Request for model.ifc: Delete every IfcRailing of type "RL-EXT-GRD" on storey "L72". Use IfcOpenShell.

First a look at what the model holds.

```python
import ifcopenshell
import ifcopenshell.util.element

model = ifcopenshell.open("model.ifc")
print(model.schema)
storey = next(s for s in model.by_type("IfcBuildingStorey") if s.Name == "L72")
railings = [e for e in ifcopenshell.util.element.get_decomposition(storey) if e.is_a("IfcRailing")]
seen = {}
for e in railings:
    element_type = ifcopenshell.util.element.get_type(e)
    name = element_type.Name if element_type not in (None, e) else None
    seen[name] = seen.get(name, 0) + 1
for name, count in sorted(seen.items(), key=str):
    print(count, "x", name)
```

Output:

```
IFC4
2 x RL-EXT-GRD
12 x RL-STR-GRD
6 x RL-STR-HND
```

```python
import ifcopenshell
import ifcopenshell.api.root
import ifcopenshell.util.element

model = ifcopenshell.open("model.ifc")

storey = next(s for s in model.by_type("IfcBuildingStorey") if s.Name == "L72")
railings = [e for e in ifcopenshell.util.element.get_decomposition(storey) if e.is_a("IfcRailing")]
targets = [e for e in railings if (t := ifcopenshell.util.element.get_type(e)) not in (None, e) and t.Name == "RL-EXT-GRD"]

for e in targets:
    ifcopenshell.api.root.remove_product(model, product=e)
print(len(targets), "removed")

model.write("model_rev.ifc")
```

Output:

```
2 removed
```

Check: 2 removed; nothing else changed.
